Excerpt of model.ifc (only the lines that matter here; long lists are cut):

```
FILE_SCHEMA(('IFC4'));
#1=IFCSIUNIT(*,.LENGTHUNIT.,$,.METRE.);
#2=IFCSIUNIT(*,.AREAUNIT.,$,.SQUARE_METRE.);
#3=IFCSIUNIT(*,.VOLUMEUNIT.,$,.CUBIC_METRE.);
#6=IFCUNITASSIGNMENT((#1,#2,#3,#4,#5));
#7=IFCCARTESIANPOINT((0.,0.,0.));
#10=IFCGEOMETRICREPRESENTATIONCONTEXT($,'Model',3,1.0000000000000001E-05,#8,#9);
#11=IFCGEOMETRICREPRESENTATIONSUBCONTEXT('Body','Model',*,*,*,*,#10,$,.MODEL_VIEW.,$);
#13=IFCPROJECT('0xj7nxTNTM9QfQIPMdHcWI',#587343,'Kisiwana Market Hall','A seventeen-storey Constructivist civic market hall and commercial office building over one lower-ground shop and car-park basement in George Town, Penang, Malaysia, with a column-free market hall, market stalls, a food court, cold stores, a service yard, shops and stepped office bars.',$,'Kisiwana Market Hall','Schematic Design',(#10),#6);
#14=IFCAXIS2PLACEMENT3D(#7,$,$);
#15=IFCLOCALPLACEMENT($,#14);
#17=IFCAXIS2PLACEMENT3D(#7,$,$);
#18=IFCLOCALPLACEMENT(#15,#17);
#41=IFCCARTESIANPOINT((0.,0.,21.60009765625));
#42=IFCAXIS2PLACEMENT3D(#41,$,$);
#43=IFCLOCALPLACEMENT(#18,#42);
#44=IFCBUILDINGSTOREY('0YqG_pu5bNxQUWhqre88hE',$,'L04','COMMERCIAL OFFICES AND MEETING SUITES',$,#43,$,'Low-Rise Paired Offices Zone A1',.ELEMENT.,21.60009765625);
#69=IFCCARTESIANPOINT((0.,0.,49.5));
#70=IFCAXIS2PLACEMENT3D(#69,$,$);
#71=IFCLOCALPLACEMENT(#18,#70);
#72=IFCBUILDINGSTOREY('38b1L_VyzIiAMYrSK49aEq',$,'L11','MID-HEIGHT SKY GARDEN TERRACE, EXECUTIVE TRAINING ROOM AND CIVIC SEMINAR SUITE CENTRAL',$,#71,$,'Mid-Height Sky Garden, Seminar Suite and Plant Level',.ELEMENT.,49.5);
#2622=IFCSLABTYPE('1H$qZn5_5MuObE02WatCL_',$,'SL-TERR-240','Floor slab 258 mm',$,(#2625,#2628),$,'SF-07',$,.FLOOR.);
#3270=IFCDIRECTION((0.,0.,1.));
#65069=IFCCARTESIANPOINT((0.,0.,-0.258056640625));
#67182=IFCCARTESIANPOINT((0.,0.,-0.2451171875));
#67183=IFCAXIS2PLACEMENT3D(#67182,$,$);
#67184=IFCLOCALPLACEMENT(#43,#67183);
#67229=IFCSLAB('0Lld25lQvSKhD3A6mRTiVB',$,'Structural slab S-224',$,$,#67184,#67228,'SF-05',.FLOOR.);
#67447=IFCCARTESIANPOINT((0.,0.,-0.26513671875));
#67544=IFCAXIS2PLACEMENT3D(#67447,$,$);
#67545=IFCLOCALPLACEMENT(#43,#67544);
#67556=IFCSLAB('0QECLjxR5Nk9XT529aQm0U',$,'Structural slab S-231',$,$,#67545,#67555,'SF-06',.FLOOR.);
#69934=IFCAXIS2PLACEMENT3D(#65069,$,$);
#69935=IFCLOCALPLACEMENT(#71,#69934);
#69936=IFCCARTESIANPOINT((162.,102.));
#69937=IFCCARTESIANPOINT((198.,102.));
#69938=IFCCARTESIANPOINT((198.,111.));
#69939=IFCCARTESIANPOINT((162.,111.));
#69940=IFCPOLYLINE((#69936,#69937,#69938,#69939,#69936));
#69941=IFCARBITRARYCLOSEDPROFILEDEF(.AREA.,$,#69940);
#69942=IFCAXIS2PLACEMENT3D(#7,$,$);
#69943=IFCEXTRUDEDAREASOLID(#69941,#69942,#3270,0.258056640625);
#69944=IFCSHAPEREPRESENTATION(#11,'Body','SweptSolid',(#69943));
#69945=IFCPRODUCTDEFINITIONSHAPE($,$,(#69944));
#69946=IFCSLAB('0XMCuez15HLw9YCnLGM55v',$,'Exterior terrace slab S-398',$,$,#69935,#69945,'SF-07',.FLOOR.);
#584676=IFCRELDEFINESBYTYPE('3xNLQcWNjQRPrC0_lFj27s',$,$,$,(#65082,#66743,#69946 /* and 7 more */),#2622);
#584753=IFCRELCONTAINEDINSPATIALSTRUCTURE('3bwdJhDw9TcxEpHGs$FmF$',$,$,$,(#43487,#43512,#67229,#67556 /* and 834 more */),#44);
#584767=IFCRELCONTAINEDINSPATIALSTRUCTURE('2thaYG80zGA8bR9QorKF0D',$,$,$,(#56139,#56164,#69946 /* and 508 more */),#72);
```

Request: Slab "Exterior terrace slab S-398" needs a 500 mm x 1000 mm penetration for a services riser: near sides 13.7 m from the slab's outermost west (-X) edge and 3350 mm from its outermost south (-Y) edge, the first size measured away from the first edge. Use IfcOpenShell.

```python
import numpy as np
import ifcopenshell
import ifcopenshell.api.feature
import ifcopenshell.api.geometry
import ifcopenshell.api.root
import ifcopenshell.geom
import ifcopenshell.util.placement
import ifcopenshell.util.representation
import ifcopenshell.util.shape
import ifcopenshell.util.unit

model = ifcopenshell.open("model.ifc")
unit_scale = ifcopenshell.util.unit.calculate_unit_scale(model)
settings = ifcopenshell.geom.settings()


def volume(element):
    """Net volume in cubic metres, openings subtracted."""
    shape = ifcopenshell.geom.create_shape(settings, element)
    return ifcopenshell.util.shape.get_volume(shape.geometry)


slab = model.by_guid("0XMCuez15HLw9YCnLGM55v")
before = volume(slab)

# Extent in the slab's own axes, in metres. The edges named are its -X and -Y sides.
slab_shape = ifcopenshell.geom.create_shape(settings, slab)
vertices = ifcopenshell.util.shape.get_vertices(slab_shape.geometry)
x_min, y_min, bottom = vertices.min(axis=0)
top = vertices[:, 2].max()

opening = ifcopenshell.api.root.create_entity(model, ifc_class="IfcOpeningElement", name="Services riser opening", predefined_type="OPENING")
context = ifcopenshell.util.representation.get_context(model, "Model", "Body", "MODEL_VIEW")
width, depth = 0.5, 1
outline = [(0.0, 0.0), (width, 0.0), (width, depth), (0.0, depth), (0.0, 0.0)]
# Overshoot both faces by 50 mm so the cut is clean.
shape = ifcopenshell.api.geometry.add_slab_representation(
    model, context=context, depth=top - bottom + 0.1, polyline=outline
)
ifcopenshell.api.geometry.assign_representation(model, product=opening, representation=shape)

matrix = ifcopenshell.util.placement.get_local_placement(slab.ObjectPlacement)
matrix[:, 3] = matrix @ np.append(np.array([x_min + 13.7, y_min + 3.35, bottom - 0.05]) / unit_scale, 1.0)
ifcopenshell.api.geometry.edit_object_placement(model, product=opening, matrix=matrix, is_si=False)
ifcopenshell.api.feature.add_feature(model, feature=opening, element=slab)

after = volume(slab)

print(f"slab volume {before:.3f} -> {after:.3f} m3")

model.write("model_v2.ifc")
```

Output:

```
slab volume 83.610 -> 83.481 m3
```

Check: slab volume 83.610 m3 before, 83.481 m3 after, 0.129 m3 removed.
